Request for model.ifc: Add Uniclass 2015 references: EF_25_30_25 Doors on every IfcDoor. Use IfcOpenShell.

First a look at what the model holds.

```python
import ifcopenshell

model = ifcopenshell.open("model.ifc")
print(model.schema)
print("classifications:", [c.Name for c in model.by_type("IfcClassification")])
for ifc_class in ("IfcDoor", "IfcRoof", "IfcStair", "IfcWall", "IfcWindow"):
    print(ifc_class, len(model.by_type(ifc_class)))
```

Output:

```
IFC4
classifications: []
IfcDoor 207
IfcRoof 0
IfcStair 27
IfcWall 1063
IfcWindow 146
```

```python
import ifcopenshell
import ifcopenshell.api.classification

model = ifcopenshell.open("model.ifc")

system = ifcopenshell.api.classification.add_classification(model, classification="Uniclass 2015")

codes = {
    "IfcDoor": ("EF_25_30_25", "Doors"),
}
for ifc_class, (code, name) in codes.items():
    products = model.by_type(ifc_class)
    ifcopenshell.api.classification.add_reference(
        model, products=products, classification=system, identification=code, name=name
    )
    print(code, len(products))

model.write("model_v2.ifc")
```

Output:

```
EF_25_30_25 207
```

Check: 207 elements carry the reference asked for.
